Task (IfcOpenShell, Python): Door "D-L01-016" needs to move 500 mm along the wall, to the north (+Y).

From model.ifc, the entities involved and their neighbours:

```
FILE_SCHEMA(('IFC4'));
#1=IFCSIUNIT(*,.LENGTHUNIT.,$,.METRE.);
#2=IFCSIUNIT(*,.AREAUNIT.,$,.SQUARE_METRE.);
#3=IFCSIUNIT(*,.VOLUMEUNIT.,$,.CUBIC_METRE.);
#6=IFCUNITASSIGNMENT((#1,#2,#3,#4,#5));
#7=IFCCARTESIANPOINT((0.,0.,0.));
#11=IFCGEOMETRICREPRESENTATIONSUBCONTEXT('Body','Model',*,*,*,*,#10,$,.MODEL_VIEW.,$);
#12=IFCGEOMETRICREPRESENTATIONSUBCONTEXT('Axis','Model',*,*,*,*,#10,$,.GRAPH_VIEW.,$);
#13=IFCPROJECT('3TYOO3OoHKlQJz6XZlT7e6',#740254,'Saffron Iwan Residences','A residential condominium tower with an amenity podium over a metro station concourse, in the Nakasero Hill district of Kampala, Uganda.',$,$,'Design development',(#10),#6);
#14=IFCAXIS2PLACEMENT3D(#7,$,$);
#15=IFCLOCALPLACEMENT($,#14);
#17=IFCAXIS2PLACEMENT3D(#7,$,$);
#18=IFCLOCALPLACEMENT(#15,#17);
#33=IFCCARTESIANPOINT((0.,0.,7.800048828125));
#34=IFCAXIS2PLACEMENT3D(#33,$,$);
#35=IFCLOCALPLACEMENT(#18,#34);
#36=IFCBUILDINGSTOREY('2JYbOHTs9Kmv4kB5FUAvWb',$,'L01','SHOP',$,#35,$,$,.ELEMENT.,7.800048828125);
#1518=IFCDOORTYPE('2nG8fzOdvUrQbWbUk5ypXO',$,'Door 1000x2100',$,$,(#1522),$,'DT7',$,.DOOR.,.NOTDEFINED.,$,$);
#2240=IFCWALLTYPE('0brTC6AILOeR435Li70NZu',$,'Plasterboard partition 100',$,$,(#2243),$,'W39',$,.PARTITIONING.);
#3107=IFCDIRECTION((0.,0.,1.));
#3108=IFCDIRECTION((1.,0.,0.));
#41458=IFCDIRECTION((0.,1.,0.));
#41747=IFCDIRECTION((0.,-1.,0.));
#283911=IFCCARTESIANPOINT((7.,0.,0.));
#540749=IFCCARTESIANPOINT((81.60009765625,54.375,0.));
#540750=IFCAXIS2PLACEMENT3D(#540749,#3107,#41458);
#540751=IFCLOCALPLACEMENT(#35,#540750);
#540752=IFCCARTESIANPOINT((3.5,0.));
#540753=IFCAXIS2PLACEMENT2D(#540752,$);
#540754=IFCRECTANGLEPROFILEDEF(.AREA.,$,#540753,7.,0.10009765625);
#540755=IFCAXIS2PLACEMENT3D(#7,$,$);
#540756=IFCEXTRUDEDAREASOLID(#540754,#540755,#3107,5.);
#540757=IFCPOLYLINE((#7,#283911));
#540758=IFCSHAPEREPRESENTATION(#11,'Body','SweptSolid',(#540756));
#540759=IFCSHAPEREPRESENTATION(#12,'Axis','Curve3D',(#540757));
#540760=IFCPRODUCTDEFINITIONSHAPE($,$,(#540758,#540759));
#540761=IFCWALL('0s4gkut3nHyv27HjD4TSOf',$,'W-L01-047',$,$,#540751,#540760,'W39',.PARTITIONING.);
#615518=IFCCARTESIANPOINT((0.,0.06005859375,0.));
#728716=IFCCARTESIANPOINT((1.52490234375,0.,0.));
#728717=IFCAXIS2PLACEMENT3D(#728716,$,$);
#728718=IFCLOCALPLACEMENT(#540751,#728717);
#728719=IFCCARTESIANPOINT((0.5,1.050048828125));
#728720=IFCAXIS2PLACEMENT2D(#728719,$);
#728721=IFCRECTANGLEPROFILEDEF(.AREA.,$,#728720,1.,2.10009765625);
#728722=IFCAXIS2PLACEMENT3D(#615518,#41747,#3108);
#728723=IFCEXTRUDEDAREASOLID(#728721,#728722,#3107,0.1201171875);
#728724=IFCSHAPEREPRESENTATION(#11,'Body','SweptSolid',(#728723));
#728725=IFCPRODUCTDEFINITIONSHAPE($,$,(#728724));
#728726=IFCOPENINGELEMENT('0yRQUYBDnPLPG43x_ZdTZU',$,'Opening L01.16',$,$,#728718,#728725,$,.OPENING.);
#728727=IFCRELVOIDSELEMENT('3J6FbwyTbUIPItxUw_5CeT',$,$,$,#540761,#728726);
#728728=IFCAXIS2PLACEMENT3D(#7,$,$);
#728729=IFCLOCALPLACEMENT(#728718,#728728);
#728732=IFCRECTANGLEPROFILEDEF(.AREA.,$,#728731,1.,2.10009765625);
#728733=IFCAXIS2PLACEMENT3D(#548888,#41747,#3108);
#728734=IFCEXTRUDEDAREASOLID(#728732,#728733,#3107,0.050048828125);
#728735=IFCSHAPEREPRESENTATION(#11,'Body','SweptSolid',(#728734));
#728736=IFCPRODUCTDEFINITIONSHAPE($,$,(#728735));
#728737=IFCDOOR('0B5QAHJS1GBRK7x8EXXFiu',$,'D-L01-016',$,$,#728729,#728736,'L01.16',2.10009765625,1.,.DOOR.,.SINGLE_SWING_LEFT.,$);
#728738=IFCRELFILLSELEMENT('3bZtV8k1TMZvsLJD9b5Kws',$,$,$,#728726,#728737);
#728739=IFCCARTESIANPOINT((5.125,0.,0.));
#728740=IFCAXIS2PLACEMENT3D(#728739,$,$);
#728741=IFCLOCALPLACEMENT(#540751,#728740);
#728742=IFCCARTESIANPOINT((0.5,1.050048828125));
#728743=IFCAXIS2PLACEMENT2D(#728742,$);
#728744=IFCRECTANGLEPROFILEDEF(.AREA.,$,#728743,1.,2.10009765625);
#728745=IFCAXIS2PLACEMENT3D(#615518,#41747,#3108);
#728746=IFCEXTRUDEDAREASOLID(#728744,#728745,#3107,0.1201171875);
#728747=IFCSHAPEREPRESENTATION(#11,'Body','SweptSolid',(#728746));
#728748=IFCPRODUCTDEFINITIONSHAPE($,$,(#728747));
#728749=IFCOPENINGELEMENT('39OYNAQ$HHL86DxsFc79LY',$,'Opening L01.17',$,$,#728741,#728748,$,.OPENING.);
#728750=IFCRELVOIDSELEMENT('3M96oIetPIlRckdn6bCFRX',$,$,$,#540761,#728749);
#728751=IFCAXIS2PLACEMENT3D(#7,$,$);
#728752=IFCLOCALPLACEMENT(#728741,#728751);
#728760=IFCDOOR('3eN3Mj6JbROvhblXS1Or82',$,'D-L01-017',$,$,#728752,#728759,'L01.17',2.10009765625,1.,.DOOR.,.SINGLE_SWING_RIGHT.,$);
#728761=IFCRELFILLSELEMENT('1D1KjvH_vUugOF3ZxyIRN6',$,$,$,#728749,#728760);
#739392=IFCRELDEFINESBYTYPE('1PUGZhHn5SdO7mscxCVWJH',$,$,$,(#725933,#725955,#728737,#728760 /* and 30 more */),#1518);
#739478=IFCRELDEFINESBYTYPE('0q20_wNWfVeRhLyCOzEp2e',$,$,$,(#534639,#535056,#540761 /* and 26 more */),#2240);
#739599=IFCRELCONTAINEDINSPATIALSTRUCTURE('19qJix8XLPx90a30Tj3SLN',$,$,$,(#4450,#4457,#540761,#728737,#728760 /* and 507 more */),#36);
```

```python
import ifcopenshell
import ifcopenshell.api.geometry
import ifcopenshell.util.placement

model = ifcopenshell.open("model.ifc")

door = model.by_id(728737)
opening = door.FillsVoids[0].RelatingOpeningElement
wall = opening.VoidsElements[0].RelatingBuildingElement

wall_matrix = ifcopenshell.util.placement.get_local_placement(wall.ObjectPlacement)
shift = wall_matrix[:3, 0] * 0.5
before = ifcopenshell.util.placement.get_local_placement(door.ObjectPlacement)[:3, 3].copy()

# The door is placed relative to its opening, so it follows when the opening moves.
matrix = ifcopenshell.util.placement.get_local_placement(opening.ObjectPlacement)
matrix[:3, 3] += shift
ifcopenshell.api.geometry.edit_object_placement(
    model, product=opening, matrix=matrix, is_si=False, should_transform_children=True
)

after = ifcopenshell.util.placement.get_local_placement(door.ObjectPlacement)[:3, 3]
print("door moved by", (after - before).round(3) + 0.0)

model.write("model_v2.ifc")
```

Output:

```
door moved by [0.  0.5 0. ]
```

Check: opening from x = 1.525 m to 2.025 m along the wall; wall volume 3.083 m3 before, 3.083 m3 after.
